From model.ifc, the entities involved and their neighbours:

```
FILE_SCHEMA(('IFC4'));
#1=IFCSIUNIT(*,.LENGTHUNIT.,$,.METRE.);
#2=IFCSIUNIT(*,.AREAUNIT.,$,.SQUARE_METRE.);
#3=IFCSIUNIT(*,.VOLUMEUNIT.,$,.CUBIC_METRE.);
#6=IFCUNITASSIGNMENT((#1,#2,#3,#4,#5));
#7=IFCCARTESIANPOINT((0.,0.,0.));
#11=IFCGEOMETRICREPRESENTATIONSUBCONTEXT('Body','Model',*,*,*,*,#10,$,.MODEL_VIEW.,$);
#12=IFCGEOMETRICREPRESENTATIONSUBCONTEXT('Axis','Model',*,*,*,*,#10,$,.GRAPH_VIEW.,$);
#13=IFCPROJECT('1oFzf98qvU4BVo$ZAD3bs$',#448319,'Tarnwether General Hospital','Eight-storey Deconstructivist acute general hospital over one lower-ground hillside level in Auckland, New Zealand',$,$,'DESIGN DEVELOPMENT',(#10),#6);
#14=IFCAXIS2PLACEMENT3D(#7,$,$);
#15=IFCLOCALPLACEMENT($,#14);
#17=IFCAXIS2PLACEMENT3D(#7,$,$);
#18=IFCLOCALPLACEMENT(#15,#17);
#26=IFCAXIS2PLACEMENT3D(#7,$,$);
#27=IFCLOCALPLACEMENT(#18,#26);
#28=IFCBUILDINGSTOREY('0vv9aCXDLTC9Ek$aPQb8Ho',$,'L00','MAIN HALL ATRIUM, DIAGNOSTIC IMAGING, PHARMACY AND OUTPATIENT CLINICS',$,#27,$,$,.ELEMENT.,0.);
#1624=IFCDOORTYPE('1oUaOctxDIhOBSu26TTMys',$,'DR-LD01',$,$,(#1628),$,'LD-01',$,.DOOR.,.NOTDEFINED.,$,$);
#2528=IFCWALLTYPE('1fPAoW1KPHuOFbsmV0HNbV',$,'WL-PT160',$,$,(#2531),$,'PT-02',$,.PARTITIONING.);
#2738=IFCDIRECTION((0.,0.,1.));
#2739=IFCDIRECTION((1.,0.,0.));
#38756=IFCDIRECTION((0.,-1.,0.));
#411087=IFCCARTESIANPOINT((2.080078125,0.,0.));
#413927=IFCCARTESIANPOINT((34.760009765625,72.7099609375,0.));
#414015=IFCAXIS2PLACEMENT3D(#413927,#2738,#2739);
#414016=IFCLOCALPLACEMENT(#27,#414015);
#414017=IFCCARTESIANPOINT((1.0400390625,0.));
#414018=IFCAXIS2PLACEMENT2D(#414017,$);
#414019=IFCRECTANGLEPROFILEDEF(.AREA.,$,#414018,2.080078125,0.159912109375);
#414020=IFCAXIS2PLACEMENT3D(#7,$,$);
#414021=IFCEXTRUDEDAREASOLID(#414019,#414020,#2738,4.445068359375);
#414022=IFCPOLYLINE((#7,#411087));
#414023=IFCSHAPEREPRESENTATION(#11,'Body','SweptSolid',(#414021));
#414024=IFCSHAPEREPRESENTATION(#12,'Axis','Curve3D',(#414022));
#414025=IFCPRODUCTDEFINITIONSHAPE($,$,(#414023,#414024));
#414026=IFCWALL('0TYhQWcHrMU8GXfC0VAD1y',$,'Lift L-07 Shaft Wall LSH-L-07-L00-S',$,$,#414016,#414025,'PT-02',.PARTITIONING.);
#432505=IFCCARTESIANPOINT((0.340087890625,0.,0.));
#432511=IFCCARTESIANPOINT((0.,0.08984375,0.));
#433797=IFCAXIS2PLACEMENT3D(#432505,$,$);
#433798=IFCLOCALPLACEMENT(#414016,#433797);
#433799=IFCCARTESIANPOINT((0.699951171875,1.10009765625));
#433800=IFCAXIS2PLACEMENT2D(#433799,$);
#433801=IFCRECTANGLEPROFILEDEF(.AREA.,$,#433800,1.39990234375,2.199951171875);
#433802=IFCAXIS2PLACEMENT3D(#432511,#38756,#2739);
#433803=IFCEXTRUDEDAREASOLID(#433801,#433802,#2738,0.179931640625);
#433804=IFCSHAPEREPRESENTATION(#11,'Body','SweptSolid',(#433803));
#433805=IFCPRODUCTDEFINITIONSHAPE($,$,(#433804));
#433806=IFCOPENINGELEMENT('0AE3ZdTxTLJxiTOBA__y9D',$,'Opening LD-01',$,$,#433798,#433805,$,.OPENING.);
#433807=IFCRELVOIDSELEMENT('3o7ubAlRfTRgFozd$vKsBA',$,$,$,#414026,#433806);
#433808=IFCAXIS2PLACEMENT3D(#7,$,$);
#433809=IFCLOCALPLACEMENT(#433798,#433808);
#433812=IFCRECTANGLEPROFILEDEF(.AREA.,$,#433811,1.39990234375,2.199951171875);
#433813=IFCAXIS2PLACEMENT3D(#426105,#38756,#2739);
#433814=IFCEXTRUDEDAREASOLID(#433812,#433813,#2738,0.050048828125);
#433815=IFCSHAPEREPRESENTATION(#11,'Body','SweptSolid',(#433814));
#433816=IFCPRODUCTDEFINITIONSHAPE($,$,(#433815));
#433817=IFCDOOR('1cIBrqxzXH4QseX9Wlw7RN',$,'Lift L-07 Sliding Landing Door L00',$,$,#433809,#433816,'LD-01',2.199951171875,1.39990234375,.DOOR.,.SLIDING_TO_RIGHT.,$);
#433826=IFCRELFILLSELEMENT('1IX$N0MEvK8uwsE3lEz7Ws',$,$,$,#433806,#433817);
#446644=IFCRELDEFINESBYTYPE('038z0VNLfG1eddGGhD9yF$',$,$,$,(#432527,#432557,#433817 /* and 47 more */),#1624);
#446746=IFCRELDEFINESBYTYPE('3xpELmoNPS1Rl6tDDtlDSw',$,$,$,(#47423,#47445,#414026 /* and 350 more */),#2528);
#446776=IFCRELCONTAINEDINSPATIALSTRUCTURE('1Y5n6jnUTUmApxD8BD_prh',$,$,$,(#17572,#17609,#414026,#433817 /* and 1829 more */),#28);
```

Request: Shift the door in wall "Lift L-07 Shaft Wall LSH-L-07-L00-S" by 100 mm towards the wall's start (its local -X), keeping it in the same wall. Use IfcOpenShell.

```python
import ifcopenshell
import ifcopenshell.api.geometry
import ifcopenshell.util.placement
import ifcopenshell.util.unit

model = ifcopenshell.open("model.ifc")
unit_scale = ifcopenshell.util.unit.calculate_unit_scale(model)

door = model.by_id(433817)
opening = door.FillsVoids[0].RelatingOpeningElement
wall = opening.VoidsElements[0].RelatingBuildingElement

wall_matrix = ifcopenshell.util.placement.get_local_placement(wall.ObjectPlacement)
shift = wall_matrix[:3, 0] * -0.1 / unit_scale
before = ifcopenshell.util.placement.get_local_placement(door.ObjectPlacement)[:3, 3].copy()

# The door is placed relative to its opening, so it follows when the opening moves.
matrix = ifcopenshell.util.placement.get_local_placement(opening.ObjectPlacement)
matrix[:3, 3] += shift
ifcopenshell.api.geometry.edit_object_placement(
    model, product=opening, matrix=matrix, is_si=False, should_transform_children=True
)

after = ifcopenshell.util.placement.get_local_placement(door.ObjectPlacement)[:3, 3]
print("door moved by", (after - before).round(3) + 0.0)

model.write("model_v2.ifc")
```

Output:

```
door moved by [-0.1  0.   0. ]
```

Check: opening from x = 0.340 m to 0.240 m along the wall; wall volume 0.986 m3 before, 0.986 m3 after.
